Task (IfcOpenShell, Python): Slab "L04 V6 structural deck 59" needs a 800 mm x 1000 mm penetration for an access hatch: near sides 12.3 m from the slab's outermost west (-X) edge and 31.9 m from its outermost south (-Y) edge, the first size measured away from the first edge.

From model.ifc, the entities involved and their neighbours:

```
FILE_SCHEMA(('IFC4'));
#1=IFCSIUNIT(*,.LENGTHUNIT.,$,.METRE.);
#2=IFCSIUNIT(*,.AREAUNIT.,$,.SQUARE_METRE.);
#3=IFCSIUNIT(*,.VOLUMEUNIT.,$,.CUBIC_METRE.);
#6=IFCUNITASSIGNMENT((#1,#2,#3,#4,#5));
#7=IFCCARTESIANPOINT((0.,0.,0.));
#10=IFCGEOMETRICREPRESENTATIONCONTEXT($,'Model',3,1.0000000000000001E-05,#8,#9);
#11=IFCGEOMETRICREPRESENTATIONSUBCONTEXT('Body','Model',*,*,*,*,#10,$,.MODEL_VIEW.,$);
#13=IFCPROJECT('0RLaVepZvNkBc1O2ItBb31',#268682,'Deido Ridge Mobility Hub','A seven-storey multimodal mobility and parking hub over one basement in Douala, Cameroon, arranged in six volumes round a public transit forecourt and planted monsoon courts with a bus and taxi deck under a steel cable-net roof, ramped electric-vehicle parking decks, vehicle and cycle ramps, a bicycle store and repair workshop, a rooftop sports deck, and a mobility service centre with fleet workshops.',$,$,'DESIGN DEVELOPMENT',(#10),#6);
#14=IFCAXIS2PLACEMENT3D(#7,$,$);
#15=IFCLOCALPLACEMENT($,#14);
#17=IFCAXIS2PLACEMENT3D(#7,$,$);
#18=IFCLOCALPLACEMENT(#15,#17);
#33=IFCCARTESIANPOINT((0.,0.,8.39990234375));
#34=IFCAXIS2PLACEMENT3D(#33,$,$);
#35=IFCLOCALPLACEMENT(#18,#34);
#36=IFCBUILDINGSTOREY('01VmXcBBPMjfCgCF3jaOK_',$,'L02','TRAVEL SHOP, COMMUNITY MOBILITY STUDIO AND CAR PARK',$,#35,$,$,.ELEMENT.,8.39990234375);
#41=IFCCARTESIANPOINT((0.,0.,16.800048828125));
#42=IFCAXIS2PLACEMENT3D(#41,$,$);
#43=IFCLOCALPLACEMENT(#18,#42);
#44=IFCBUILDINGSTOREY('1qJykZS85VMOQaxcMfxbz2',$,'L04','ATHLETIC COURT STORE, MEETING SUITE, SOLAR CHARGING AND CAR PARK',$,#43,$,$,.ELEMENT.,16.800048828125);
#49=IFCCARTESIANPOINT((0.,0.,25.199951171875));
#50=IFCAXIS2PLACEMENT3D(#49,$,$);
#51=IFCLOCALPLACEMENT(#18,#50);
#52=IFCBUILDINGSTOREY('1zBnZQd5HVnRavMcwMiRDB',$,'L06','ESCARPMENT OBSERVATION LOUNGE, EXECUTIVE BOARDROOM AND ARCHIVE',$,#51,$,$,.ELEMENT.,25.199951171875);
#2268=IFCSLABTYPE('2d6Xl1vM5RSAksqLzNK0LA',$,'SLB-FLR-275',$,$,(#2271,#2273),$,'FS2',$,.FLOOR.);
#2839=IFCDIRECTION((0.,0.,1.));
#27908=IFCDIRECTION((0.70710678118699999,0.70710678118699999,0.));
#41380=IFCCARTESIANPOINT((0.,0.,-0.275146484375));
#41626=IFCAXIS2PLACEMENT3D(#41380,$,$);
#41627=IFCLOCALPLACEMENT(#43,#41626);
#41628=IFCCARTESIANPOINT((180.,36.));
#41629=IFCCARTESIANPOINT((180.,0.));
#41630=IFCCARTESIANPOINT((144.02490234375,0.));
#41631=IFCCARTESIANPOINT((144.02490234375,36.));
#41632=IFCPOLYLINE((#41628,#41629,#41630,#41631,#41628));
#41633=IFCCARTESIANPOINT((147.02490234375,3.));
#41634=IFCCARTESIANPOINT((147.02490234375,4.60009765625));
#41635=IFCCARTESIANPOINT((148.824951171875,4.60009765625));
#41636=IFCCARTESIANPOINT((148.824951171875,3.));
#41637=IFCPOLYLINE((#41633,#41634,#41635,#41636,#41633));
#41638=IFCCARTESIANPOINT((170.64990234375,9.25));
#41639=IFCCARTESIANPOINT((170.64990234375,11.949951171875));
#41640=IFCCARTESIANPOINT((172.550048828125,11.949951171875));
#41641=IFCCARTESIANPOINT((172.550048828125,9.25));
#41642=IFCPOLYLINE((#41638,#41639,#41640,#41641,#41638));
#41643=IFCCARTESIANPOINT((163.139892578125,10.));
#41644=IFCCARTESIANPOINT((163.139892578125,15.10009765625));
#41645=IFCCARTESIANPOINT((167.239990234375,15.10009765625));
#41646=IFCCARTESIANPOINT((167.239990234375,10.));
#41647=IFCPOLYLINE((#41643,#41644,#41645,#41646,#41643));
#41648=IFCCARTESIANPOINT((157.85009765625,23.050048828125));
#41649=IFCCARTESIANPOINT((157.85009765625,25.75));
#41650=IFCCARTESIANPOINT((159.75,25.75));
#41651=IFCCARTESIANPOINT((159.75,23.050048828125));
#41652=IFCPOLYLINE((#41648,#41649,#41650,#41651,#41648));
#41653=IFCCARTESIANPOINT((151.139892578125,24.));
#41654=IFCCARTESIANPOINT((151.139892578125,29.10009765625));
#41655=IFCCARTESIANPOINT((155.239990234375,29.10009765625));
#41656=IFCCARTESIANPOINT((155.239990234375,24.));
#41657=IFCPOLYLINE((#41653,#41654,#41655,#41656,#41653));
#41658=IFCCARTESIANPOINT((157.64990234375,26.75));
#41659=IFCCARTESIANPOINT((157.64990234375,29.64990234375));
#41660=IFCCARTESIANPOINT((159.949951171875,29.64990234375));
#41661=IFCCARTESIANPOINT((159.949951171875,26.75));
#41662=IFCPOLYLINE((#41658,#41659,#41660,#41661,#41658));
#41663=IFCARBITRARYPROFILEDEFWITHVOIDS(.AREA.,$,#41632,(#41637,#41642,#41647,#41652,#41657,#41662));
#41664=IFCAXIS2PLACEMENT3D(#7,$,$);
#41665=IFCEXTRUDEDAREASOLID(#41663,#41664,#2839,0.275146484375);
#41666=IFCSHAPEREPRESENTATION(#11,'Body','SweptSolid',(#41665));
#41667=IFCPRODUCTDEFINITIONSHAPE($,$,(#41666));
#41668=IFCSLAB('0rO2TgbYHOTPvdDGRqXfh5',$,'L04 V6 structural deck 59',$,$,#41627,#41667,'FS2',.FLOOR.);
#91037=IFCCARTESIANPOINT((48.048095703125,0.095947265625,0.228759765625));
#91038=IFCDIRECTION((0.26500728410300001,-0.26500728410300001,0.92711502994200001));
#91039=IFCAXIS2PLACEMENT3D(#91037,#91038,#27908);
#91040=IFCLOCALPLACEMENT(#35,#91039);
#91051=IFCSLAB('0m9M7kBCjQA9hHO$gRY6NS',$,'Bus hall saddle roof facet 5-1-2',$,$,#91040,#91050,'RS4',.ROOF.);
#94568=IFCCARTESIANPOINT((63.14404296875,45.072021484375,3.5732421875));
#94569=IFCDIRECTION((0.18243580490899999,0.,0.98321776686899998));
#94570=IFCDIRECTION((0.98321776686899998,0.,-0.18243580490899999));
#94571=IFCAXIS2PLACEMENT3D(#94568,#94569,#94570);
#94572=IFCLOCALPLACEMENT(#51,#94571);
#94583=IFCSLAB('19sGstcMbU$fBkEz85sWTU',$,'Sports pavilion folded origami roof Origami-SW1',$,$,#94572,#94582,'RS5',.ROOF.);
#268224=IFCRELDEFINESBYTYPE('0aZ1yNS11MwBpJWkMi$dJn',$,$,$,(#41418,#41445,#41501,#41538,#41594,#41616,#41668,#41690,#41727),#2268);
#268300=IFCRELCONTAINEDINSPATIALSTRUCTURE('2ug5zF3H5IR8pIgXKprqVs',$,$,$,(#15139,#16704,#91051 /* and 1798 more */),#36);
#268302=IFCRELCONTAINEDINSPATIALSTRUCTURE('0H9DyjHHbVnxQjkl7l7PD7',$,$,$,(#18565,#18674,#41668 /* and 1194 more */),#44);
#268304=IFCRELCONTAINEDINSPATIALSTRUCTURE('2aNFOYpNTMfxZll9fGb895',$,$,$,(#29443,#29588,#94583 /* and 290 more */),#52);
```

```python
import numpy as np
import ifcopenshell
import ifcopenshell.api.feature
import ifcopenshell.api.geometry
import ifcopenshell.api.root
import ifcopenshell.geom
import ifcopenshell.util.placement
import ifcopenshell.util.representation
import ifcopenshell.util.shape
import ifcopenshell.util.unit

model = ifcopenshell.open("model.ifc")
unit_scale = ifcopenshell.util.unit.calculate_unit_scale(model)
settings = ifcopenshell.geom.settings()


def volume(element):
    """Net volume in cubic metres, openings subtracted."""
    shape = ifcopenshell.geom.create_shape(settings, element)
    return ifcopenshell.util.shape.get_volume(shape.geometry)


slab = model.by_guid("0rO2TgbYHOTPvdDGRqXfh5")
before = volume(slab)

# Extent in the slab's own axes, in metres. The edges named are its -X and -Y sides.
slab_shape = ifcopenshell.geom.create_shape(settings, slab)
vertices = ifcopenshell.util.shape.get_vertices(slab_shape.geometry)
x_min, y_min, bottom = vertices.min(axis=0)
top = vertices[:, 2].max()

opening = ifcopenshell.api.root.create_entity(model, ifc_class="IfcOpeningElement", name="Access hatch opening", predefined_type="OPENING")
context = ifcopenshell.util.representation.get_context(model, "Model", "Body", "MODEL_VIEW")
width, depth = 0.8, 1
outline = [(0.0, 0.0), (width, 0.0), (width, depth), (0.0, depth), (0.0, 0.0)]
# Overshoot both faces by 50 mm so the cut is clean.
shape = ifcopenshell.api.geometry.add_slab_representation(
    model, context=context, depth=top - bottom + 0.1, polyline=outline
)
ifcopenshell.api.geometry.assign_representation(model, product=opening, representation=shape)

matrix = ifcopenshell.util.placement.get_local_placement(slab.ObjectPlacement)
matrix[:, 3] = matrix @ np.append(np.array([x_min + 12.3, y_min + 31.9, bottom - 0.05]) / unit_scale, 1.0)
ifcopenshell.api.geometry.edit_object_placement(model, product=opening, matrix=matrix, is_si=False)
ifcopenshell.api.feature.add_feature(model, feature=opening, element=slab)

after = volume(slab)

print(f"slab volume {before:.3f} -> {after:.3f} m3")

model.write("model_v2.ifc")
```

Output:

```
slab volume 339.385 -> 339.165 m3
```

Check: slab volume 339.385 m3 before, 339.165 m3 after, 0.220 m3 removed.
